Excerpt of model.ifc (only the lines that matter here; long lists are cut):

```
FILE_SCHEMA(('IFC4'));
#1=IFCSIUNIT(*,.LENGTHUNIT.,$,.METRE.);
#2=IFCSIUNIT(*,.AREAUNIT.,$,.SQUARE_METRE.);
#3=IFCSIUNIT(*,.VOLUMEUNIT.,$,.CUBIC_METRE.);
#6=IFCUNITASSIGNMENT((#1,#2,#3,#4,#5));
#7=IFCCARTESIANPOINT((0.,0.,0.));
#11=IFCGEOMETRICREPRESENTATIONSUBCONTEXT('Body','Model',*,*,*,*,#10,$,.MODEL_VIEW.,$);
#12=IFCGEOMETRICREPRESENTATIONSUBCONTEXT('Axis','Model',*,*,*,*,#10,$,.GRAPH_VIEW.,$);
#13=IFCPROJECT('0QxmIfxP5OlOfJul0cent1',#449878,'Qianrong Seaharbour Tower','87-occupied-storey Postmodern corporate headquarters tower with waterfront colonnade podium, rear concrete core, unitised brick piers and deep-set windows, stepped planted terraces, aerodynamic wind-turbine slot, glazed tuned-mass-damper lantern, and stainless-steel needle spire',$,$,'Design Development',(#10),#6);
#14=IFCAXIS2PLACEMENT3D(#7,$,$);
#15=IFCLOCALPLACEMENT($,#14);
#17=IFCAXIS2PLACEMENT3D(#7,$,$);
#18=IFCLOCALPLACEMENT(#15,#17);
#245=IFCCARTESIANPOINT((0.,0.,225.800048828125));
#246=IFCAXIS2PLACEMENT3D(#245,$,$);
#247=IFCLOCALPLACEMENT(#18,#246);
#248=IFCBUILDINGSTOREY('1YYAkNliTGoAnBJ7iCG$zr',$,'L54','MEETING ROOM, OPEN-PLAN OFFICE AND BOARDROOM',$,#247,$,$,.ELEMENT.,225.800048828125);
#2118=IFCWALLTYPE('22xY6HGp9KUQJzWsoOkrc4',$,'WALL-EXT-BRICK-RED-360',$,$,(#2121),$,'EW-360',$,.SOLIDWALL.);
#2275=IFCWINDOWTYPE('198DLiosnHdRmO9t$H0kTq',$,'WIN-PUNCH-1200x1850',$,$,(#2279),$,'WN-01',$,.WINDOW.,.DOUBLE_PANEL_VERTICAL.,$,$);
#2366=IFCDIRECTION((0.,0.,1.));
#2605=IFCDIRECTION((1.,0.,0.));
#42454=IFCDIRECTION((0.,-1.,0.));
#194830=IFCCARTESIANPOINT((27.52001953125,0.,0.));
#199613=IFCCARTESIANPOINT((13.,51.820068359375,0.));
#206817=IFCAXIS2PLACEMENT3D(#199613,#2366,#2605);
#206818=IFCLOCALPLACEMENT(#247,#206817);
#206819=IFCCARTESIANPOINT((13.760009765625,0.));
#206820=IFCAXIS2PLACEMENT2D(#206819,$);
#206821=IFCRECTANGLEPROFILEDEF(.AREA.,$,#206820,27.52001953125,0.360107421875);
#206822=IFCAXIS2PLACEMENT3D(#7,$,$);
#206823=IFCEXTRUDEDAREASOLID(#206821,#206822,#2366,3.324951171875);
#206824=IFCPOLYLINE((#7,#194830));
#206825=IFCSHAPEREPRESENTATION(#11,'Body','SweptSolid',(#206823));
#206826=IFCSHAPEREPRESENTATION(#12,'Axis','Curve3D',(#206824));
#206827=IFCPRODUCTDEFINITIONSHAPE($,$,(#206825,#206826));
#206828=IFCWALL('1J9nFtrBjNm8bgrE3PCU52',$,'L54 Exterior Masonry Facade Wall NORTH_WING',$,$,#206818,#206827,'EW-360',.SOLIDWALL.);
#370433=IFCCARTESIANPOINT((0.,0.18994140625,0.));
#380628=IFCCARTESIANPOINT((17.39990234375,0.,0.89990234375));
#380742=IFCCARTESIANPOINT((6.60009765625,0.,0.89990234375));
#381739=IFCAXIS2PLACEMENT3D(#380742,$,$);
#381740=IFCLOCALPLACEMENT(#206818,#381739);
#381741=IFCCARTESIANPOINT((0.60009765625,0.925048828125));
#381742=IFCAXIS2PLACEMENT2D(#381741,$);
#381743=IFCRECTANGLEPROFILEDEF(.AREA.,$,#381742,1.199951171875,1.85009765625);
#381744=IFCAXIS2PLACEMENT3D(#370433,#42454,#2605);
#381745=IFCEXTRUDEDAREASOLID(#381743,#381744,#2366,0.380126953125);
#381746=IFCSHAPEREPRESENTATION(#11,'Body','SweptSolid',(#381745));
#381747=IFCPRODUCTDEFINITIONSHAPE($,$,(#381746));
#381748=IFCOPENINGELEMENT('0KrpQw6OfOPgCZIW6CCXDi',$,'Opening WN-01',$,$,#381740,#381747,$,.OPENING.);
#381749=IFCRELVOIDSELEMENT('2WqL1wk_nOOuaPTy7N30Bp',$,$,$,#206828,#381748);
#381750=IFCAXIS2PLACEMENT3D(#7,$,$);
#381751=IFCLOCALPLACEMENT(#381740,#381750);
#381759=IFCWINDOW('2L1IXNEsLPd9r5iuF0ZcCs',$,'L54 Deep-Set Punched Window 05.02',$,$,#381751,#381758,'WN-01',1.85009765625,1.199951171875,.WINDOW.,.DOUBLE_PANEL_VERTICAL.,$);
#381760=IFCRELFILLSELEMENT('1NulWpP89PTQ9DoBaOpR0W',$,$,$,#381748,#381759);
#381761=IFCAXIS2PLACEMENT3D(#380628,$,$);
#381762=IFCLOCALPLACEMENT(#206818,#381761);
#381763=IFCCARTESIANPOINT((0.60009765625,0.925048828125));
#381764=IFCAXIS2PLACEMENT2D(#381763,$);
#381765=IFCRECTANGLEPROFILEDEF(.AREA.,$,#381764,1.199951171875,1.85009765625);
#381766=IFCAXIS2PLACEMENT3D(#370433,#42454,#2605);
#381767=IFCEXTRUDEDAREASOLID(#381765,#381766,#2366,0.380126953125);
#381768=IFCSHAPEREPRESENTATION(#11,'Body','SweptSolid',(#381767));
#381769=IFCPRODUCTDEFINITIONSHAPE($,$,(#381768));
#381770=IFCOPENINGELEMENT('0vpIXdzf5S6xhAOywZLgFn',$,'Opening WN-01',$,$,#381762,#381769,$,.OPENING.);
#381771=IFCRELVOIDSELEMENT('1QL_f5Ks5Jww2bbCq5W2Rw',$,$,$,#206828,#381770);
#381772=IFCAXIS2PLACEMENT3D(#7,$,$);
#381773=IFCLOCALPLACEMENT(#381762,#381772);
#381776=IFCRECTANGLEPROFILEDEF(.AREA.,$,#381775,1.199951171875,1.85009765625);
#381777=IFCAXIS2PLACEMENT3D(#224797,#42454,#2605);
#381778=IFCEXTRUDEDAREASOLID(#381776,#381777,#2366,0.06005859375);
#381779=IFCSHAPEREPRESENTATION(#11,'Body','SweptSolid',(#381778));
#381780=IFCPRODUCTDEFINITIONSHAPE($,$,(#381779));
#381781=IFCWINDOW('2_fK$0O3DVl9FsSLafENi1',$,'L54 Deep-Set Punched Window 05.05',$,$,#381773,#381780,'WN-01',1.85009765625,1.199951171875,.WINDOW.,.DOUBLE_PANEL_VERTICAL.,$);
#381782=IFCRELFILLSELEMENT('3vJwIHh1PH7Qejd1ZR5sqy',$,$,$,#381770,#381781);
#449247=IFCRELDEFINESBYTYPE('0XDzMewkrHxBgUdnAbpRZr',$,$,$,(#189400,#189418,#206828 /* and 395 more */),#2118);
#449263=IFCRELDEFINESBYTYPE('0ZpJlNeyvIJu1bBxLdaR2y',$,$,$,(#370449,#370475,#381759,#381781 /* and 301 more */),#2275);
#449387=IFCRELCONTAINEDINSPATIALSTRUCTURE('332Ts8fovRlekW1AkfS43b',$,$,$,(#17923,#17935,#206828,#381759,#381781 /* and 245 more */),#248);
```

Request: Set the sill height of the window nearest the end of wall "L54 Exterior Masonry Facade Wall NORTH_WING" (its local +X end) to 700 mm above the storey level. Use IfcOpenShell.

```python
import numpy as np
import ifcopenshell
import ifcopenshell.api.geometry
import ifcopenshell.geom
import ifcopenshell.util.element
import ifcopenshell.util.placement
import ifcopenshell.util.shape
import ifcopenshell.util.unit

model = ifcopenshell.open("model.ifc")
unit_scale = ifcopenshell.util.unit.calculate_unit_scale(model)

window = model.by_id(381781)
opening = window.FillsVoids[0].RelatingOpeningElement
storey = ifcopenshell.util.element.get_container(window, ifc_class="IfcBuildingStorey")
level = ifcopenshell.util.placement.get_local_placement(storey.ObjectPlacement)[2, 3]

# The opening's origin need not be at the sill, so measure its lowest point.
shape = ifcopenshell.geom.create_shape(ifcopenshell.geom.settings(), opening)
bottom = ifcopenshell.util.shape.get_shape_bottom_elevation(shape, shape.geometry) / unit_scale
dz = level + 0.7 - bottom

shift = np.array([0.0, 0.0, dz])
# The window is placed relative to its opening, so it follows when the opening moves.
matrix = ifcopenshell.util.placement.get_local_placement(opening.ObjectPlacement)
matrix[:3, 3] += shift
ifcopenshell.api.geometry.edit_object_placement(
    model, product=opening, matrix=matrix, is_si=False, should_transform_children=True
)

print(f"moved by {dz * unit_scale:+.3f} m")

model.write("model_edited.ifc")
```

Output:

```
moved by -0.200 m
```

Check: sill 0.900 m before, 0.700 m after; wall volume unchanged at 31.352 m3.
